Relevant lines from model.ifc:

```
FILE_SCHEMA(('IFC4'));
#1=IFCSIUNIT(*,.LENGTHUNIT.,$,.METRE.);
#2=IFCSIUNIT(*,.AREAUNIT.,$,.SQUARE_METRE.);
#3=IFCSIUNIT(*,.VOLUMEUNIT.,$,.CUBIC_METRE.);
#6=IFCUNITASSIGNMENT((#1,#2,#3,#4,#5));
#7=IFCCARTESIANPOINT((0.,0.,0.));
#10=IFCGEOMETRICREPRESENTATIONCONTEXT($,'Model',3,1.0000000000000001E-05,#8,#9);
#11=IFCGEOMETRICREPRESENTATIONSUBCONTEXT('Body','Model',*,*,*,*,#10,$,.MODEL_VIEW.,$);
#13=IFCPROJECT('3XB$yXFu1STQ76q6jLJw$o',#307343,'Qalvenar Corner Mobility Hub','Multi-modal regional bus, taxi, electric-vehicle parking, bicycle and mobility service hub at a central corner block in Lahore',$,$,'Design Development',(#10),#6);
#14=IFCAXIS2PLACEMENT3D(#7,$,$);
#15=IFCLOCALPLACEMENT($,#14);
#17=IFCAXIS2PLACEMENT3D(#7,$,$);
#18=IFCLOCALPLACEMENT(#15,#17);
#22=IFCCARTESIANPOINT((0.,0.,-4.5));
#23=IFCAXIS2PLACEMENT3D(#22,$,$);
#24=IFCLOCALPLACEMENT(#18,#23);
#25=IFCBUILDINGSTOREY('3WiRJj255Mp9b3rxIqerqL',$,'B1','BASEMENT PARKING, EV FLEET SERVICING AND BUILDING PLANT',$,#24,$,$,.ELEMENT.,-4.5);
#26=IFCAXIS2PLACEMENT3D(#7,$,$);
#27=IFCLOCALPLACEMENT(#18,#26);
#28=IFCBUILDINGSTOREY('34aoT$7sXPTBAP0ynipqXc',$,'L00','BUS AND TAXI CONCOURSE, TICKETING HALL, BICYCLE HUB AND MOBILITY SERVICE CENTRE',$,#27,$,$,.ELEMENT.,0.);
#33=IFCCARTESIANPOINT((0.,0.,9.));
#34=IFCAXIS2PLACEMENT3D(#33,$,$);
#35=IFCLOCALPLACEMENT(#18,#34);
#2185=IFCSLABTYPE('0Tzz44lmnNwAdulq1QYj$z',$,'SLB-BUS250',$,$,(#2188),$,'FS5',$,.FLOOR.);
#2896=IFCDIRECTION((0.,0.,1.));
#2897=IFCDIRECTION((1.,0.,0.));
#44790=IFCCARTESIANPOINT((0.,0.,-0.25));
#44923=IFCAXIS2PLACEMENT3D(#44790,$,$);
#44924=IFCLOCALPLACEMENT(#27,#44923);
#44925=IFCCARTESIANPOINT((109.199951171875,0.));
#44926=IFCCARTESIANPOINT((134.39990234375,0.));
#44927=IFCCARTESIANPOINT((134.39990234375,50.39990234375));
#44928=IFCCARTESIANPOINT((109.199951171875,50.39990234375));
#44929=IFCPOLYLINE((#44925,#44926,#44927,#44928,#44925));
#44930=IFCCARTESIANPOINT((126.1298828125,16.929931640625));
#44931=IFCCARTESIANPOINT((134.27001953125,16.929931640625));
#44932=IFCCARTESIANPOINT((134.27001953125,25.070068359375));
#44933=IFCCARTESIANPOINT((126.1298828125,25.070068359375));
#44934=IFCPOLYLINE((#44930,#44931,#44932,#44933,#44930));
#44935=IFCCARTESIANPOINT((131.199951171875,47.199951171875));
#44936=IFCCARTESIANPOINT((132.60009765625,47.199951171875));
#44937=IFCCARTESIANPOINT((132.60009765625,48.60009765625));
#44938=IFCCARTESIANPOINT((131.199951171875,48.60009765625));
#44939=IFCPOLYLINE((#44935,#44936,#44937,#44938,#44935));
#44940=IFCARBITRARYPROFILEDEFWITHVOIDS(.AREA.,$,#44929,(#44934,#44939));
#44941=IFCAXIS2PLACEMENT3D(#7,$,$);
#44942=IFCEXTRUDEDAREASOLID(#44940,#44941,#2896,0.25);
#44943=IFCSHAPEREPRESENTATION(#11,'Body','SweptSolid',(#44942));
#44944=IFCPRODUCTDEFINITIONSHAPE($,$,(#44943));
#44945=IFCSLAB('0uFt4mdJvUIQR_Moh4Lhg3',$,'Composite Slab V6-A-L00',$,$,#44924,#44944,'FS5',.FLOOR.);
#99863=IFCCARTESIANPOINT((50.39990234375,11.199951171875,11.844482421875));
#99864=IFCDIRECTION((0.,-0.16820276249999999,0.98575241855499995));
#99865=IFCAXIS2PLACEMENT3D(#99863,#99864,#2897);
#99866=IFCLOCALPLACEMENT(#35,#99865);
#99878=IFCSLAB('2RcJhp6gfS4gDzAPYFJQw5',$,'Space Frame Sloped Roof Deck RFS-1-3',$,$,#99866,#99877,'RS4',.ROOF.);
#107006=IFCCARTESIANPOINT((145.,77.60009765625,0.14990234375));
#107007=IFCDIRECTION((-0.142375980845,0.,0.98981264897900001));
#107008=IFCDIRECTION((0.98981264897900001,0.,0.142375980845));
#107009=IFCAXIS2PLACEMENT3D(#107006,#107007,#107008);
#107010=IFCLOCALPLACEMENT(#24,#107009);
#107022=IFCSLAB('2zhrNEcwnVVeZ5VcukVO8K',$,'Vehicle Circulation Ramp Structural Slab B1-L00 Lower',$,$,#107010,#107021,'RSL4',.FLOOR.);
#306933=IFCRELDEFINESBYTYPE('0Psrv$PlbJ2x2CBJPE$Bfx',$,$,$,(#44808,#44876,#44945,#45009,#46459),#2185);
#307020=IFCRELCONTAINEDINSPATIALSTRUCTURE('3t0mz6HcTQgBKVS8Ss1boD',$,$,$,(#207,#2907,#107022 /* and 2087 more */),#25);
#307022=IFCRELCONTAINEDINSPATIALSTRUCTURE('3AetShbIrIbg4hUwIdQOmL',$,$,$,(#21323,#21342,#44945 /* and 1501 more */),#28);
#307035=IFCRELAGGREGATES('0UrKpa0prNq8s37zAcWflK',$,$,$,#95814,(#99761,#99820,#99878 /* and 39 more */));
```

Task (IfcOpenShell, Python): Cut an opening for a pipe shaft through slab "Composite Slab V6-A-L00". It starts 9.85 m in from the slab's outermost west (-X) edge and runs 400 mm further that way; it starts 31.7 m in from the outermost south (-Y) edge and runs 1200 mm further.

```python
import numpy as np
import ifcopenshell
import ifcopenshell.api.feature
import ifcopenshell.api.geometry
import ifcopenshell.api.root
import ifcopenshell.geom
import ifcopenshell.util.placement
import ifcopenshell.util.representation
import ifcopenshell.util.shape
import ifcopenshell.util.unit

model = ifcopenshell.open("model.ifc")
unit_scale = ifcopenshell.util.unit.calculate_unit_scale(model)
settings = ifcopenshell.geom.settings()


def volume(element):
    """Net volume in cubic metres, openings subtracted."""
    shape = ifcopenshell.geom.create_shape(settings, element)
    return ifcopenshell.util.shape.get_volume(shape.geometry)


slab = model.by_id(44945)
before = volume(slab)

# Extent in the slab's own axes, in metres. The edges named are its -X and -Y sides.
slab_shape = ifcopenshell.geom.create_shape(settings, slab)
vertices = ifcopenshell.util.shape.get_vertices(slab_shape.geometry)
x_min, y_min, bottom = vertices.min(axis=0)
top = vertices[:, 2].max()

opening = ifcopenshell.api.root.create_entity(model, ifc_class="IfcOpeningElement", name="Pipe shaft opening", predefined_type="OPENING")
context = ifcopenshell.util.representation.get_context(model, "Model", "Body", "MODEL_VIEW")
width, depth = 0.4, 1.2
outline = [(0.0, 0.0), (width, 0.0), (width, depth), (0.0, depth), (0.0, 0.0)]
# Overshoot both faces by 50 mm so the cut is clean.
shape = ifcopenshell.api.geometry.add_slab_representation(
    model, context=context, depth=top - bottom + 0.1, polyline=outline
)
ifcopenshell.api.geometry.assign_representation(model, product=opening, representation=shape)

matrix = ifcopenshell.util.placement.get_local_placement(slab.ObjectPlacement)
matrix[:, 3] = matrix @ np.append(np.array([x_min + 9.85, y_min + 31.7, bottom - 0.05]) / unit_scale, 1.0)
ifcopenshell.api.geometry.edit_object_placement(model, product=opening, matrix=matrix, is_si=False)
ifcopenshell.api.feature.add_feature(model, feature=opening, element=slab)

after = volume(slab)

print(f"slab volume {before:.3f} -> {after:.3f} m3")

model.write("model_edited.ifc")
```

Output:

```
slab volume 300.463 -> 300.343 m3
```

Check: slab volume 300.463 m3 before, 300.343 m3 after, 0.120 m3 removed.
